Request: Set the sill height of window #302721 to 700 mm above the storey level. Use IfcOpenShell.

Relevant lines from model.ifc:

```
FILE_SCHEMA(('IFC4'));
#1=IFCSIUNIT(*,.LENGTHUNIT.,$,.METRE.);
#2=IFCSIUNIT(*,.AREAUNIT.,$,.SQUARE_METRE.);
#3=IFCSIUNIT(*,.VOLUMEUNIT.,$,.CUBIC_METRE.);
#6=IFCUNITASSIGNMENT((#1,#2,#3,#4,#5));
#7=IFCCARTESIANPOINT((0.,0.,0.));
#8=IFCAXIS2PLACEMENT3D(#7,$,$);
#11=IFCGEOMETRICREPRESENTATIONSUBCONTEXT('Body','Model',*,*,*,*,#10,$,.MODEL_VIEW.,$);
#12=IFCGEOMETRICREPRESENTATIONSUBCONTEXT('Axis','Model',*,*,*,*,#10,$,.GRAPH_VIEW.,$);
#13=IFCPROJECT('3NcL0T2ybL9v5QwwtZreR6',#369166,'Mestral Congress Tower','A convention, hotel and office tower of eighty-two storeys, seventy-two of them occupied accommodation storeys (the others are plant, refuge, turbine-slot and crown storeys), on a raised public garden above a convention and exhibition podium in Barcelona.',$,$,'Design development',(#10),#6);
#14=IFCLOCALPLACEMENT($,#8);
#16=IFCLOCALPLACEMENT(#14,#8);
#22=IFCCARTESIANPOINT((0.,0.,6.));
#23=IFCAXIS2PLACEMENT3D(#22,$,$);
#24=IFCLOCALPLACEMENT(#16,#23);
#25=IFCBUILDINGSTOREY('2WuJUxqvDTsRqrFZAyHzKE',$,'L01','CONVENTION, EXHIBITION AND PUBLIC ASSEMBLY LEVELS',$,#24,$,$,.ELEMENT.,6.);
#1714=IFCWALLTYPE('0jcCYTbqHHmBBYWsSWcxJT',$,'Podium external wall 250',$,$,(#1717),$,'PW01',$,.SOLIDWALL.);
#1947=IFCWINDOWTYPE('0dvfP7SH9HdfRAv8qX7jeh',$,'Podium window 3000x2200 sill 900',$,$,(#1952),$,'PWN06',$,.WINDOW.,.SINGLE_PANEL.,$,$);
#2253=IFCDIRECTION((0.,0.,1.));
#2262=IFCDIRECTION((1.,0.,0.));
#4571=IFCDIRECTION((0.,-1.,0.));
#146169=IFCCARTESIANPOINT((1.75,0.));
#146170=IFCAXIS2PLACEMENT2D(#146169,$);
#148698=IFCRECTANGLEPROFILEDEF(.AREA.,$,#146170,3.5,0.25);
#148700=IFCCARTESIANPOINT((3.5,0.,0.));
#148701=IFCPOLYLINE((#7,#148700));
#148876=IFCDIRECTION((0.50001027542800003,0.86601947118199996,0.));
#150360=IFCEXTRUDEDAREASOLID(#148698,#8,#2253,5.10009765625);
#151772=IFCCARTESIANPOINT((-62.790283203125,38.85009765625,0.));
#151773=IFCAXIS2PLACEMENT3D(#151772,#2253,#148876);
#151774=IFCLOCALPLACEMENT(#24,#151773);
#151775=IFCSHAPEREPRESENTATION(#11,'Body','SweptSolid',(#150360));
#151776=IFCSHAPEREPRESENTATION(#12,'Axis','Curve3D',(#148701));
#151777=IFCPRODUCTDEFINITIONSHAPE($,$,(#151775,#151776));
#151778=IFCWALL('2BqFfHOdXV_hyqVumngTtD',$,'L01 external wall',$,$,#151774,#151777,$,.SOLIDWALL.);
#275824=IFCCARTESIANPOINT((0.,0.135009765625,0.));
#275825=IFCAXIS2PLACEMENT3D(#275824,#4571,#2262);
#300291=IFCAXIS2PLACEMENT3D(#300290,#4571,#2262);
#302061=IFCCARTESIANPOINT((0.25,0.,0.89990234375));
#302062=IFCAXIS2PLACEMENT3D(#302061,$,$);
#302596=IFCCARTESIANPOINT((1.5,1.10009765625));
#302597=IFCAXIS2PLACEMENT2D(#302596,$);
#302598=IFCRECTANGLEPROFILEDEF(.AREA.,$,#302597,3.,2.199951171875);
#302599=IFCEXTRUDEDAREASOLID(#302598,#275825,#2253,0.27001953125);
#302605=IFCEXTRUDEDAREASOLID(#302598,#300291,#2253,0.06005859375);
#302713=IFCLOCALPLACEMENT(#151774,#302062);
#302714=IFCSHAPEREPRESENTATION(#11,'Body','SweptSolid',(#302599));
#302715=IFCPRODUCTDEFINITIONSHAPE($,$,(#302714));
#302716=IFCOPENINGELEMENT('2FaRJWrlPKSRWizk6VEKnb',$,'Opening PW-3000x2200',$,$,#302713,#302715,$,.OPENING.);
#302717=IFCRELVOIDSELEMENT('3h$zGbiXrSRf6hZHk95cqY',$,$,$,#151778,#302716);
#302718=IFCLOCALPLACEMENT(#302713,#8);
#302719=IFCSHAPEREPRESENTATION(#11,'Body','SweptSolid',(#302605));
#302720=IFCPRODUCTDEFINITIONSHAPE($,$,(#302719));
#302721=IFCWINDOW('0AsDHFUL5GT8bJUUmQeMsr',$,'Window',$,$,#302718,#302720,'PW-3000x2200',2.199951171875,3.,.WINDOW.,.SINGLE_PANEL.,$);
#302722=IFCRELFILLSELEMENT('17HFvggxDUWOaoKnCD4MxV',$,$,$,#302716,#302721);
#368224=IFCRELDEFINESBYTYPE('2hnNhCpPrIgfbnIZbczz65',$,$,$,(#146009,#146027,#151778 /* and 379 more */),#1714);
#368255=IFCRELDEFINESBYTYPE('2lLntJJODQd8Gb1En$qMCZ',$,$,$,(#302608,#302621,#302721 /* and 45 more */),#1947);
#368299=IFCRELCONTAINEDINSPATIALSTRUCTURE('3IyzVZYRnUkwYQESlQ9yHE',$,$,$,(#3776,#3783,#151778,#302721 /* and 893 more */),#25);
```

```python
import numpy as np
import ifcopenshell
import ifcopenshell.api.geometry
import ifcopenshell.geom
import ifcopenshell.util.element
import ifcopenshell.util.placement
import ifcopenshell.util.shape
import ifcopenshell.util.unit

model = ifcopenshell.open("model.ifc")
unit_scale = ifcopenshell.util.unit.calculate_unit_scale(model)

window = model.by_guid("0AsDHFUL5GT8bJUUmQeMsr")
opening = window.FillsVoids[0].RelatingOpeningElement
storey = ifcopenshell.util.element.get_container(window, ifc_class="IfcBuildingStorey")
level = ifcopenshell.util.placement.get_local_placement(storey.ObjectPlacement)[2, 3]

# The opening's origin need not be at the sill, so measure its lowest point.
shape = ifcopenshell.geom.create_shape(ifcopenshell.geom.settings(), opening)
bottom = ifcopenshell.util.shape.get_shape_bottom_elevation(shape, shape.geometry) / unit_scale
dz = level + 0.7 - bottom

shift = np.array([0.0, 0.0, dz])
# The window is placed relative to its opening, so it follows when the opening moves.
matrix = ifcopenshell.util.placement.get_local_placement(opening.ObjectPlacement)
matrix[:3, 3] += shift
ifcopenshell.api.geometry.edit_object_placement(
    model, product=opening, matrix=matrix, is_si=False, should_transform_children=True
)

print(f"moved by {dz * unit_scale:+.3f} m")

model.write("model_edited.ifc")
```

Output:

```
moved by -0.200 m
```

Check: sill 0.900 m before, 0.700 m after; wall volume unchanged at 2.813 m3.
